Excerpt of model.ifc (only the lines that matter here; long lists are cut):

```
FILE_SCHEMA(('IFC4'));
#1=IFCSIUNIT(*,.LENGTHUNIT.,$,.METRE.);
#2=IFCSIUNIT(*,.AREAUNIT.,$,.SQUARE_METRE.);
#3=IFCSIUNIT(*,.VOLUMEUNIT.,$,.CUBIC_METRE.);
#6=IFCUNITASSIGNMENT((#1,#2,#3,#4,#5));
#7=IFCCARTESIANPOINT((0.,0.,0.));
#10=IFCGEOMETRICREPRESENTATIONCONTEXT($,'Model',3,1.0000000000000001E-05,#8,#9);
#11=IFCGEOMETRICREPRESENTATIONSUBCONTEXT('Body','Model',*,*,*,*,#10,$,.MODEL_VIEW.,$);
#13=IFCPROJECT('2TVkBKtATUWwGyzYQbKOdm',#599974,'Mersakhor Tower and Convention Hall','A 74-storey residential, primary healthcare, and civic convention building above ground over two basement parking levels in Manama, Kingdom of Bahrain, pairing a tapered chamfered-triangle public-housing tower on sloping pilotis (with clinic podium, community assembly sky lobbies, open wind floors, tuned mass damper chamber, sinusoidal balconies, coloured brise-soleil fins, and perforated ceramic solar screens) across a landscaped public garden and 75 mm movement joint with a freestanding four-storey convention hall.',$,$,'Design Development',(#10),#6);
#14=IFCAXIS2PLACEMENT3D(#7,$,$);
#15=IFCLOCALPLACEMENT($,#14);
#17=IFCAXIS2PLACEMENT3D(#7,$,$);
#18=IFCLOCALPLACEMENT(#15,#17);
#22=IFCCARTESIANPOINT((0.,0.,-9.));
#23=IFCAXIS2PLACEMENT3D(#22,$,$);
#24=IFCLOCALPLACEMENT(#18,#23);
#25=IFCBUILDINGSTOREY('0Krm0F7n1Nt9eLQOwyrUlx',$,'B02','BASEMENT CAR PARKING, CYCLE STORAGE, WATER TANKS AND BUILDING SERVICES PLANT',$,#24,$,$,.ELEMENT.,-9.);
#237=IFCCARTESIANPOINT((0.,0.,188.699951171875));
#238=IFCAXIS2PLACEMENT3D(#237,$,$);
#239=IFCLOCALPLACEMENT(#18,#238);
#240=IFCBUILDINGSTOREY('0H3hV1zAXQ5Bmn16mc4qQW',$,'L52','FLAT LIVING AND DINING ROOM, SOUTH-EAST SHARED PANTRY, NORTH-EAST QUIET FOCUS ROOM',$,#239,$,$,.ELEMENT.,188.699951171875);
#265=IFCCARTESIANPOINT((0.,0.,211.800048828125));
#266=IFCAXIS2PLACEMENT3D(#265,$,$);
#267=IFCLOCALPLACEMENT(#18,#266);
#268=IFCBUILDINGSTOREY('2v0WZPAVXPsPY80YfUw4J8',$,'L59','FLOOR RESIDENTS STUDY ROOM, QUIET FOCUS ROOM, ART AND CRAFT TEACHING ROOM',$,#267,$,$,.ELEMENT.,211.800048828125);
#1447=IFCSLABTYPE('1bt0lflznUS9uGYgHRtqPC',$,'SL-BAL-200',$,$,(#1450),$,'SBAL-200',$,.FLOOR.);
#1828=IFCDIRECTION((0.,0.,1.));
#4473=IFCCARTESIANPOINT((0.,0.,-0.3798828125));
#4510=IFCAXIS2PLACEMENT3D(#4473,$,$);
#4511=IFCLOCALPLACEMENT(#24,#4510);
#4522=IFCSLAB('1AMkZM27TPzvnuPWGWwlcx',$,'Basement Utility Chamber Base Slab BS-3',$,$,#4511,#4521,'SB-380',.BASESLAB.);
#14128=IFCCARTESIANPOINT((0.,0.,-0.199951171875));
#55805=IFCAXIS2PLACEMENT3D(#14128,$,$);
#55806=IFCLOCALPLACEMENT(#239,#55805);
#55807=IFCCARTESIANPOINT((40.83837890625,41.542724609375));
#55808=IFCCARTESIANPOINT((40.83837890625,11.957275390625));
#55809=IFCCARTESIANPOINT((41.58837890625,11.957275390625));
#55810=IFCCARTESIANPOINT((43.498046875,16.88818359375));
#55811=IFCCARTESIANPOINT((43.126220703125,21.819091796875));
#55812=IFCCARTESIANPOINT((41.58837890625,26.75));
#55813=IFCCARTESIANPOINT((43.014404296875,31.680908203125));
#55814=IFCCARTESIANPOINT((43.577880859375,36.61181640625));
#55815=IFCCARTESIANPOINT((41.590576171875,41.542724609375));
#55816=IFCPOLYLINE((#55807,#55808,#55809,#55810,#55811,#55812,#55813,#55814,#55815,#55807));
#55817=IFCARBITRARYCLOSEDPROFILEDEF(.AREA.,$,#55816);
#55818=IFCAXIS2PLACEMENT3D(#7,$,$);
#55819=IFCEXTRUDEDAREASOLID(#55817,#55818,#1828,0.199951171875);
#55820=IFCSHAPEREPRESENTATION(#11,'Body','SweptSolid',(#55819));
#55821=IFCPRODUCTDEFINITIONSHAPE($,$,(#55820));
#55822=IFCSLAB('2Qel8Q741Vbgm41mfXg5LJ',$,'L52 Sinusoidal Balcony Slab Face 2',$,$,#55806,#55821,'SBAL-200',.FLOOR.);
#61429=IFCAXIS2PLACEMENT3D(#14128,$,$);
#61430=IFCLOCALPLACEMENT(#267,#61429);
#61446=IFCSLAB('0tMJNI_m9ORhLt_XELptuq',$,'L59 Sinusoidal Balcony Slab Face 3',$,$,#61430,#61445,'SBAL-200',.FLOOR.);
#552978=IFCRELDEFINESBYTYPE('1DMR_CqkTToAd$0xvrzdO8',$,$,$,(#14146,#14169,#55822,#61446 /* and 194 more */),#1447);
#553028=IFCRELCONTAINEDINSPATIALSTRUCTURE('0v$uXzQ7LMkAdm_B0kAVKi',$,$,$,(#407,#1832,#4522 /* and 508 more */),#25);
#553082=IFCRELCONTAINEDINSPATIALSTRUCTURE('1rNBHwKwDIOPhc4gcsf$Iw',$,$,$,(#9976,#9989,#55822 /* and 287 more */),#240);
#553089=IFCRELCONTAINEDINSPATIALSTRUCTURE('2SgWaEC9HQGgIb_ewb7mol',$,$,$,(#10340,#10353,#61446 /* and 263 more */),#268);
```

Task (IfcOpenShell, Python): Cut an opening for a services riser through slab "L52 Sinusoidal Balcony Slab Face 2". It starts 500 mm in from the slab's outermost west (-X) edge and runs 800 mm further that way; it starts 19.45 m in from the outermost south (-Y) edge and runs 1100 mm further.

```python
import numpy as np
import ifcopenshell
import ifcopenshell.api.feature
import ifcopenshell.api.geometry
import ifcopenshell.api.root
import ifcopenshell.geom
import ifcopenshell.util.placement
import ifcopenshell.util.representation
import ifcopenshell.util.shape
import ifcopenshell.util.unit

model = ifcopenshell.open("model.ifc")
unit_scale = ifcopenshell.util.unit.calculate_unit_scale(model)
settings = ifcopenshell.geom.settings()


def volume(element):
    """Net volume in cubic metres, openings subtracted."""
    shape = ifcopenshell.geom.create_shape(settings, element)
    return ifcopenshell.util.shape.get_volume(shape.geometry)


slab = model.by_id(55822)
before = volume(slab)

# Extent in the slab's own axes, in metres. The edges named are its -X and -Y sides.
slab_shape = ifcopenshell.geom.create_shape(settings, slab)
vertices = ifcopenshell.util.shape.get_vertices(slab_shape.geometry)
x_min, y_min, bottom = vertices.min(axis=0)
top = vertices[:, 2].max()

opening = ifcopenshell.api.root.create_entity(model, ifc_class="IfcOpeningElement", name="Services riser opening", predefined_type="OPENING")
context = ifcopenshell.util.representation.get_context(model, "Model", "Body", "MODEL_VIEW")
width, depth = 0.8, 1.1
outline = [(0.0, 0.0), (width, 0.0), (width, depth), (0.0, depth), (0.0, 0.0)]
# Overshoot both faces by 50 mm so the cut is clean.
shape = ifcopenshell.api.geometry.add_slab_representation(
    model, context=context, depth=top - bottom + 0.1, polyline=outline
)
ifcopenshell.api.geometry.assign_representation(model, product=opening, representation=shape)

matrix = ifcopenshell.util.placement.get_local_placement(slab.ObjectPlacement)
matrix[:, 3] = matrix @ np.append(np.array([x_min + 0.5, y_min + 19.45, bottom - 0.05]) / unit_scale, 1.0)
ifcopenshell.api.geometry.edit_object_placement(model, product=opening, matrix=matrix, is_si=False)
ifcopenshell.api.feature.add_feature(model, feature=opening, element=slab)

after = volume(slab)

print(f"slab volume {before:.3f} -> {after:.3f} m3")

model.write("model_edited.ifc")
```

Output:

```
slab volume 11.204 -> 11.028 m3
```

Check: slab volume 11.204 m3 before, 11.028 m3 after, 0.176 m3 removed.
